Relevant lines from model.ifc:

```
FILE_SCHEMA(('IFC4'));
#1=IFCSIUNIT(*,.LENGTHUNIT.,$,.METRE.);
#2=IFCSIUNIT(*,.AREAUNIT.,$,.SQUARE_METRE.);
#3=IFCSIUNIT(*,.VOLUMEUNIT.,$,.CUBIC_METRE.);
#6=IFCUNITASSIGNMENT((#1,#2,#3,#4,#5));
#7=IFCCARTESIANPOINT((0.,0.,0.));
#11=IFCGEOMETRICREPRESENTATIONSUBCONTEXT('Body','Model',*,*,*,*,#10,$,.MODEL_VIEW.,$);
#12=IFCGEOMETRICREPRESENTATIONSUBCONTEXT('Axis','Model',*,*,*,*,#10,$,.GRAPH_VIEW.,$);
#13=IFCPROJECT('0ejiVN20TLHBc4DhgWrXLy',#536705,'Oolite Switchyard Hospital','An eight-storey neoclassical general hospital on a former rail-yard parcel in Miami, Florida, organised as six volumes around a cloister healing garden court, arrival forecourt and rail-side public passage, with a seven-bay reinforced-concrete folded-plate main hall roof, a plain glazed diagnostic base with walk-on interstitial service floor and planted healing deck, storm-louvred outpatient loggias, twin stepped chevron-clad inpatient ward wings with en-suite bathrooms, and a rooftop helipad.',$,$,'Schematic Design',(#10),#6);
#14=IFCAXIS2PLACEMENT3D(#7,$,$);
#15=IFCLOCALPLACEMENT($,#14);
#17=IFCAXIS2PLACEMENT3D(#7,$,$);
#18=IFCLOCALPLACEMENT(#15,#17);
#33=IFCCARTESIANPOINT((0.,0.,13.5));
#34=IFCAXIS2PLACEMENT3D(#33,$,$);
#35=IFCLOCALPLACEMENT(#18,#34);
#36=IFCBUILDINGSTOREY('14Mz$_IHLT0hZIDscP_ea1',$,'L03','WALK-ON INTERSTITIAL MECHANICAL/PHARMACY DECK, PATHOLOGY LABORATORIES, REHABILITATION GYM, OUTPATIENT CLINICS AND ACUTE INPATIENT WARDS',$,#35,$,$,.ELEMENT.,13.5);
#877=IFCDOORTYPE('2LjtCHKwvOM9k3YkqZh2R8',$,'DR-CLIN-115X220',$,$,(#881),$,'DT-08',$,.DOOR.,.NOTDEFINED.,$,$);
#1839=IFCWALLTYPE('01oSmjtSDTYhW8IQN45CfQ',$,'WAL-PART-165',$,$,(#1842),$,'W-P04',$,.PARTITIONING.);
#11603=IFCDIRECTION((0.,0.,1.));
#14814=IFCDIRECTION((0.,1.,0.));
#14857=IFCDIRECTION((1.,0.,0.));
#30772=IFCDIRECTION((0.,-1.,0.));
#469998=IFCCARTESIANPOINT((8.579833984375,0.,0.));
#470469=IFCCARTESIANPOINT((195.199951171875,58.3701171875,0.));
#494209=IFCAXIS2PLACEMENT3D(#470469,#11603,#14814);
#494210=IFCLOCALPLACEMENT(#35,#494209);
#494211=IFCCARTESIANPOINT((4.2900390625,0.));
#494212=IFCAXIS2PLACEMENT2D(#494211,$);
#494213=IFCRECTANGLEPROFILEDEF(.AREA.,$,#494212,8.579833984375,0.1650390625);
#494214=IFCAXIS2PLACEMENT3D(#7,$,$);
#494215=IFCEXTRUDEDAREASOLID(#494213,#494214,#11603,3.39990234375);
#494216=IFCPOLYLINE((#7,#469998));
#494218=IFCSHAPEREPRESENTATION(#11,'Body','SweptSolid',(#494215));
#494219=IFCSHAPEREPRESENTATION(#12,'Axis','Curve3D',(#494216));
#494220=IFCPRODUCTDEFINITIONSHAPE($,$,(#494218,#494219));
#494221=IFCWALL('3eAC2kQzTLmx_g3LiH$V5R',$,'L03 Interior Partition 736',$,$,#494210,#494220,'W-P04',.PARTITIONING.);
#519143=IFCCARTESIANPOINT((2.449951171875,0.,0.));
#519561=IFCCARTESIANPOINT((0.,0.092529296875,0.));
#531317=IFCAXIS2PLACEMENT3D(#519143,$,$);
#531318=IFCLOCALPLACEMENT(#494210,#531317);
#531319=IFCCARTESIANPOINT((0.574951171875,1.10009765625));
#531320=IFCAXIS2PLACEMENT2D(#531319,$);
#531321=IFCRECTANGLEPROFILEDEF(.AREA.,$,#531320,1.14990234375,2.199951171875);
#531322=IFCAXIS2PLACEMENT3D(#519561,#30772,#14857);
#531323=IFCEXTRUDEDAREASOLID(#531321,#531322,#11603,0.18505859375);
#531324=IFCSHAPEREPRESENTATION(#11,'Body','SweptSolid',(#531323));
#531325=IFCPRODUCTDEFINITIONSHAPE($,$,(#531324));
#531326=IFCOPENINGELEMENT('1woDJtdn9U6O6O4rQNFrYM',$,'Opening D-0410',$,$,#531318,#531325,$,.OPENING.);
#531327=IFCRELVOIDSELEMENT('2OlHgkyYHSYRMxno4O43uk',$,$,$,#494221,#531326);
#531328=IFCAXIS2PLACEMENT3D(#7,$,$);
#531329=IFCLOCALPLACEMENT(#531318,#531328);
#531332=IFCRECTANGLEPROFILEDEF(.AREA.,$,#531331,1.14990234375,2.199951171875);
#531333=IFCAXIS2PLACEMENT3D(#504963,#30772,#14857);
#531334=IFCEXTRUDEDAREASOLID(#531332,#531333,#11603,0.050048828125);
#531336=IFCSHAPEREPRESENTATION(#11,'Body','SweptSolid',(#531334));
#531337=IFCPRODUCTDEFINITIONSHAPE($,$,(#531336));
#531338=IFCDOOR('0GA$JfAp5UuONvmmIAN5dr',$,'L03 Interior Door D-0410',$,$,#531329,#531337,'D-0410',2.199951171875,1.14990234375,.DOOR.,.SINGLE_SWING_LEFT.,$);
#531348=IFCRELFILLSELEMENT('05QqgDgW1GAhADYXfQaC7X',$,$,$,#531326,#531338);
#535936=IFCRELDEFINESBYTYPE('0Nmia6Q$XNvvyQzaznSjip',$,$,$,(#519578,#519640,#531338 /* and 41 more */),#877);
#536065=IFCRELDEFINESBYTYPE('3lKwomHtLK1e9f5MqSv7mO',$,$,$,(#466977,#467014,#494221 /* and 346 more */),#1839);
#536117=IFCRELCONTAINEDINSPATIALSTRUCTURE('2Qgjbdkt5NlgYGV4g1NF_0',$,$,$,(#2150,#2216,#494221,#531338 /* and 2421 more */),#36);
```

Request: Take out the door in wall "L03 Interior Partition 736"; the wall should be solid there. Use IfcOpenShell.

```python
import ifcopenshell
import ifcopenshell.api.feature
import ifcopenshell.api.root
import ifcopenshell.geom
import ifcopenshell.util.shape

model = ifcopenshell.open("model.ifc")
settings = ifcopenshell.geom.settings()


def volume(element):
    """Net volume in cubic metres, openings subtracted."""
    shape = ifcopenshell.geom.create_shape(settings, element)
    return ifcopenshell.util.shape.get_volume(shape.geometry)


door = model.by_guid("0GA$JfAp5UuONvmmIAN5dr")
opening = door.FillsVoids[0].RelatingOpeningElement
wall = opening.VoidsElements[0].RelatingBuildingElement
before = volume(wall)

ifcopenshell.api.root.remove_product(model, product=door)
ifcopenshell.api.feature.remove_feature(model, feature=opening)

after = volume(wall)

print(f"wall volume {before:.3f} -> {after:.3f} m3")

model.write("model_updated.ifc")
```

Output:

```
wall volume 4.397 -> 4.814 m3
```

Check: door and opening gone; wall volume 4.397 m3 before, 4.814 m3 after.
